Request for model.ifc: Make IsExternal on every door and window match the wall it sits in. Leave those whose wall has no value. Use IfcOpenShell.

First a look at what the model holds.

```python
import ifcopenshell
import ifcopenshell.util.element

model = ifcopenshell.open("model.ifc")
print(model.schema)
seen = {}
for e in model.by_type("IfcDoor") + model.by_type("IfcWindow"):
    if not e.FillsVoids:
        continue
    host = e.FillsVoids[0].RelatingOpeningElement.VoidsElements[0].RelatingBuildingElement
    own = ifcopenshell.util.element.get_pset(e, f"Pset_{e.is_a()[3:].removesuffix('StandardCase')}Common", "IsExternal")
    wall = ifcopenshell.util.element.get_pset(host, "Pset_WallCommon", "IsExternal")
    seen[e.is_a(), own, wall] = seen.get((e.is_a(), own, wall), 0) + 1
for (cls, own, wall), count in sorted(seen.items(), key=str):
    print(count, cls, "IsExternal:", own, "| host wall:", wall)
```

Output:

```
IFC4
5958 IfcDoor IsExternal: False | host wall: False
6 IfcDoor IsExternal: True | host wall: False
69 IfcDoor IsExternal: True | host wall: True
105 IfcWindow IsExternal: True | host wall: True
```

```python
import ifcopenshell
import ifcopenshell.api.pset
import ifcopenshell.util.element

model = ifcopenshell.open("model.ifc")

count = 0
for ifc_class, pset_name in (("IfcDoor", "Pset_DoorCommon"), ("IfcWindow", "Pset_WindowCommon")):
    for e in model.by_type(ifc_class):
        if not e.FillsVoids:
            continue
        host = e.FillsVoids[0].RelatingOpeningElement.VoidsElements[0].RelatingBuildingElement
        external = ifcopenshell.util.element.get_pset(host, "Pset_WallCommon", "IsExternal")
        if external is None or ifcopenshell.util.element.get_pset(e, pset_name, "IsExternal") == external:
            continue
        pset = ifcopenshell.api.pset.add_pset(model, product=e, name=pset_name)
        ifcopenshell.api.pset.edit_pset(model, pset=pset, properties={"IsExternal": external})
        count += 1

print(count, "updated")

model.write("model_v2.ifc")
```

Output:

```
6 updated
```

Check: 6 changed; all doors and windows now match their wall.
